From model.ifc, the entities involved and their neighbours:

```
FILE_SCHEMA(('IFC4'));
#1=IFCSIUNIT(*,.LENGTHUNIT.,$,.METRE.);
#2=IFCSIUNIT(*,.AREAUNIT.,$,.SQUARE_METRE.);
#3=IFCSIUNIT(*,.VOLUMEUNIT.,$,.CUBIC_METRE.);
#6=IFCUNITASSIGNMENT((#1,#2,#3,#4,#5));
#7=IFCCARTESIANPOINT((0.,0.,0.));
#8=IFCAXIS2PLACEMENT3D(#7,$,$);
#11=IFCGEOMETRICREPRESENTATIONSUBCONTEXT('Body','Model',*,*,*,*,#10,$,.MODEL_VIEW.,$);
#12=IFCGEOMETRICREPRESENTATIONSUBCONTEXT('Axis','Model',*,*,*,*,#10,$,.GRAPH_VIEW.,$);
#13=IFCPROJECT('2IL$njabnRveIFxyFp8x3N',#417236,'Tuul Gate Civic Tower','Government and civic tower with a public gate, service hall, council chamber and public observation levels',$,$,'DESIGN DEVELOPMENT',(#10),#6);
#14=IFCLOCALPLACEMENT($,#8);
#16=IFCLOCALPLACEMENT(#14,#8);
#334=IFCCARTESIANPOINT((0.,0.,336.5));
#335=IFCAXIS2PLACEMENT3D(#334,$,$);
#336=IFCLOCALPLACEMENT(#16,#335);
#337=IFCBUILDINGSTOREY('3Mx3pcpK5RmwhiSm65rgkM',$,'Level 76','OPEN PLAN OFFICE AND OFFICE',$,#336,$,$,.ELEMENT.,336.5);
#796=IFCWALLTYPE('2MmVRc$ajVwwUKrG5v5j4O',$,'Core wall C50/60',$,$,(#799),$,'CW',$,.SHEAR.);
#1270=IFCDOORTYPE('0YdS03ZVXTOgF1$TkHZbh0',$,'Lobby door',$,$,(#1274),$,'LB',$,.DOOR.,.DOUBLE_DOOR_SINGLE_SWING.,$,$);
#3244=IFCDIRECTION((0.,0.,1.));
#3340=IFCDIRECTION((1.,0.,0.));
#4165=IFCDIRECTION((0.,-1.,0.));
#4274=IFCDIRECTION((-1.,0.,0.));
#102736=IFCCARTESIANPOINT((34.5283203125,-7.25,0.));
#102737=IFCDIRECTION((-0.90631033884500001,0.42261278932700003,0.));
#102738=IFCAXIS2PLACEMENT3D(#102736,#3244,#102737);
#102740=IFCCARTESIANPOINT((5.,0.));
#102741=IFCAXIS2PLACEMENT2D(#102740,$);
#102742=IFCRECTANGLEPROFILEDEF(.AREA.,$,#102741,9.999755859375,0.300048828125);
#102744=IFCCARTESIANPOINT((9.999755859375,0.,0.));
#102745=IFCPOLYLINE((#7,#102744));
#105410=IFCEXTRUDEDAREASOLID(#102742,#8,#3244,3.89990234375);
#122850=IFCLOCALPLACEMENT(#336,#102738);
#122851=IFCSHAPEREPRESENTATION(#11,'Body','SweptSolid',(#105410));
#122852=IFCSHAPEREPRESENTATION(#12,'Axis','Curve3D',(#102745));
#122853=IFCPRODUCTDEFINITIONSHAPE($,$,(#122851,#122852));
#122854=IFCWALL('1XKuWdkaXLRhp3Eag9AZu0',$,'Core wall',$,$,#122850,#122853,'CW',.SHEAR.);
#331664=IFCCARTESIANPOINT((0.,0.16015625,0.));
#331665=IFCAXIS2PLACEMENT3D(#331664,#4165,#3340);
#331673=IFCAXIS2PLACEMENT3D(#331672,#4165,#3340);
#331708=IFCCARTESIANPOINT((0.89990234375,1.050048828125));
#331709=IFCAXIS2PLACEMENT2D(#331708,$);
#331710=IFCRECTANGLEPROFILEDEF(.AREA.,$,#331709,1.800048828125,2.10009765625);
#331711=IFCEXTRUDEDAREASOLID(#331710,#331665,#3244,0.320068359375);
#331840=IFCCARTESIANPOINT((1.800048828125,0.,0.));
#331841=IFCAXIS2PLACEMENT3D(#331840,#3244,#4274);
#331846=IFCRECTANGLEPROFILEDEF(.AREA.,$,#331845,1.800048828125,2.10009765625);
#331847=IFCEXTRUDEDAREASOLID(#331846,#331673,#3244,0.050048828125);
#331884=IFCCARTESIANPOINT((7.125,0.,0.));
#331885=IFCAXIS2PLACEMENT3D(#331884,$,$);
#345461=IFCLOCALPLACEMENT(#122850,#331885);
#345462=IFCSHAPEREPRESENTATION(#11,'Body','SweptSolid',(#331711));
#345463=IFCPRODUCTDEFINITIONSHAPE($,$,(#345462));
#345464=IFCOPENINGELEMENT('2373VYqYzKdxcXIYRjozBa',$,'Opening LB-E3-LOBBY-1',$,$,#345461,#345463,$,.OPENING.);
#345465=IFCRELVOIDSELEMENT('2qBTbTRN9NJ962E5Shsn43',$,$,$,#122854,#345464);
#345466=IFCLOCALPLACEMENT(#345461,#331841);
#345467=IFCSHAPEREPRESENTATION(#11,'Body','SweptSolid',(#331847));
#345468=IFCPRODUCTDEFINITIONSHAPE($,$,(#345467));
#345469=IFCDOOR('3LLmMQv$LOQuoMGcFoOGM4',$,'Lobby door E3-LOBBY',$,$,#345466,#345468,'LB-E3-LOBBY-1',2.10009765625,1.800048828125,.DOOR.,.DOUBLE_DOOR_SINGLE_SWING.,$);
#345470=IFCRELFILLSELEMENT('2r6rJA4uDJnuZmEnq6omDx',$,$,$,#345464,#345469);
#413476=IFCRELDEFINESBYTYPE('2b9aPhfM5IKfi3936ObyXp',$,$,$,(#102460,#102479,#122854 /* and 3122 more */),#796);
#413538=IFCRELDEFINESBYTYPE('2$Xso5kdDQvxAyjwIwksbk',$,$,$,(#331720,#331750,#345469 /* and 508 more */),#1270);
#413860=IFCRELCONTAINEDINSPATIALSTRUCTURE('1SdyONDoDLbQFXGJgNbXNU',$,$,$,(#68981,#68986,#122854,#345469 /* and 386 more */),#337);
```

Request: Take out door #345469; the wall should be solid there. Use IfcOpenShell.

```python
import ifcopenshell
import ifcopenshell.api.feature
import ifcopenshell.api.root
import ifcopenshell.geom
import ifcopenshell.util.shape

model = ifcopenshell.open("model.ifc")
settings = ifcopenshell.geom.settings()


def volume(element):
    """Net volume in cubic metres, openings subtracted."""
    shape = ifcopenshell.geom.create_shape(settings, element)
    return ifcopenshell.util.shape.get_volume(shape.geometry)


door = model.by_guid("3LLmMQv$LOQuoMGcFoOGM4")
opening = door.FillsVoids[0].RelatingOpeningElement
wall = opening.VoidsElements[0].RelatingBuildingElement
before = volume(wall)

ifcopenshell.api.root.remove_product(model, product=door)
ifcopenshell.api.feature.remove_feature(model, feature=opening)

after = volume(wall)

print(f"wall volume {before:.3f} -> {after:.3f} m3")

model.write("model_rev.ifc")
```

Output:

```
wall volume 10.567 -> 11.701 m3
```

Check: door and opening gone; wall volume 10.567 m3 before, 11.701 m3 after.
